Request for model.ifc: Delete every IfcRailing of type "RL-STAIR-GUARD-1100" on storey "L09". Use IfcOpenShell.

First a look at what the model holds.

```python
import ifcopenshell
import ifcopenshell.util.element

model = ifcopenshell.open("model.ifc")
print(model.schema)
storey = next(s for s in model.by_type("IfcBuildingStorey") if s.Name == "L09")
railings = [e for e in ifcopenshell.util.element.get_decomposition(storey) if e.is_a("IfcRailing")]
seen = {}
for e in railings:
    element_type = ifcopenshell.util.element.get_type(e)
    name = element_type.Name if element_type not in (None, e) else None
    seen[name] = seen.get(name, 0) + 1
for name, count in sorted(seen.items(), key=str):
    print(count, "x", name)
```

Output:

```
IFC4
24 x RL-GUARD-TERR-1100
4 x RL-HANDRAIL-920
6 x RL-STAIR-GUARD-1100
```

```python
import ifcopenshell
import ifcopenshell.api.root
import ifcopenshell.util.element

model = ifcopenshell.open("model.ifc")

storey = next(s for s in model.by_type("IfcBuildingStorey") if s.Name == "L09")
railings = [e for e in ifcopenshell.util.element.get_decomposition(storey) if e.is_a("IfcRailing")]
targets = [e for e in railings if (t := ifcopenshell.util.element.get_type(e)) not in (None, e) and t.Name == "RL-STAIR-GUARD-1100"]

for e in targets:
    ifcopenshell.api.root.remove_product(model, product=e)
print(len(targets), "removed")

model.write("model_edited.ifc")
```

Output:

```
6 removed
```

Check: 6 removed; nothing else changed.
